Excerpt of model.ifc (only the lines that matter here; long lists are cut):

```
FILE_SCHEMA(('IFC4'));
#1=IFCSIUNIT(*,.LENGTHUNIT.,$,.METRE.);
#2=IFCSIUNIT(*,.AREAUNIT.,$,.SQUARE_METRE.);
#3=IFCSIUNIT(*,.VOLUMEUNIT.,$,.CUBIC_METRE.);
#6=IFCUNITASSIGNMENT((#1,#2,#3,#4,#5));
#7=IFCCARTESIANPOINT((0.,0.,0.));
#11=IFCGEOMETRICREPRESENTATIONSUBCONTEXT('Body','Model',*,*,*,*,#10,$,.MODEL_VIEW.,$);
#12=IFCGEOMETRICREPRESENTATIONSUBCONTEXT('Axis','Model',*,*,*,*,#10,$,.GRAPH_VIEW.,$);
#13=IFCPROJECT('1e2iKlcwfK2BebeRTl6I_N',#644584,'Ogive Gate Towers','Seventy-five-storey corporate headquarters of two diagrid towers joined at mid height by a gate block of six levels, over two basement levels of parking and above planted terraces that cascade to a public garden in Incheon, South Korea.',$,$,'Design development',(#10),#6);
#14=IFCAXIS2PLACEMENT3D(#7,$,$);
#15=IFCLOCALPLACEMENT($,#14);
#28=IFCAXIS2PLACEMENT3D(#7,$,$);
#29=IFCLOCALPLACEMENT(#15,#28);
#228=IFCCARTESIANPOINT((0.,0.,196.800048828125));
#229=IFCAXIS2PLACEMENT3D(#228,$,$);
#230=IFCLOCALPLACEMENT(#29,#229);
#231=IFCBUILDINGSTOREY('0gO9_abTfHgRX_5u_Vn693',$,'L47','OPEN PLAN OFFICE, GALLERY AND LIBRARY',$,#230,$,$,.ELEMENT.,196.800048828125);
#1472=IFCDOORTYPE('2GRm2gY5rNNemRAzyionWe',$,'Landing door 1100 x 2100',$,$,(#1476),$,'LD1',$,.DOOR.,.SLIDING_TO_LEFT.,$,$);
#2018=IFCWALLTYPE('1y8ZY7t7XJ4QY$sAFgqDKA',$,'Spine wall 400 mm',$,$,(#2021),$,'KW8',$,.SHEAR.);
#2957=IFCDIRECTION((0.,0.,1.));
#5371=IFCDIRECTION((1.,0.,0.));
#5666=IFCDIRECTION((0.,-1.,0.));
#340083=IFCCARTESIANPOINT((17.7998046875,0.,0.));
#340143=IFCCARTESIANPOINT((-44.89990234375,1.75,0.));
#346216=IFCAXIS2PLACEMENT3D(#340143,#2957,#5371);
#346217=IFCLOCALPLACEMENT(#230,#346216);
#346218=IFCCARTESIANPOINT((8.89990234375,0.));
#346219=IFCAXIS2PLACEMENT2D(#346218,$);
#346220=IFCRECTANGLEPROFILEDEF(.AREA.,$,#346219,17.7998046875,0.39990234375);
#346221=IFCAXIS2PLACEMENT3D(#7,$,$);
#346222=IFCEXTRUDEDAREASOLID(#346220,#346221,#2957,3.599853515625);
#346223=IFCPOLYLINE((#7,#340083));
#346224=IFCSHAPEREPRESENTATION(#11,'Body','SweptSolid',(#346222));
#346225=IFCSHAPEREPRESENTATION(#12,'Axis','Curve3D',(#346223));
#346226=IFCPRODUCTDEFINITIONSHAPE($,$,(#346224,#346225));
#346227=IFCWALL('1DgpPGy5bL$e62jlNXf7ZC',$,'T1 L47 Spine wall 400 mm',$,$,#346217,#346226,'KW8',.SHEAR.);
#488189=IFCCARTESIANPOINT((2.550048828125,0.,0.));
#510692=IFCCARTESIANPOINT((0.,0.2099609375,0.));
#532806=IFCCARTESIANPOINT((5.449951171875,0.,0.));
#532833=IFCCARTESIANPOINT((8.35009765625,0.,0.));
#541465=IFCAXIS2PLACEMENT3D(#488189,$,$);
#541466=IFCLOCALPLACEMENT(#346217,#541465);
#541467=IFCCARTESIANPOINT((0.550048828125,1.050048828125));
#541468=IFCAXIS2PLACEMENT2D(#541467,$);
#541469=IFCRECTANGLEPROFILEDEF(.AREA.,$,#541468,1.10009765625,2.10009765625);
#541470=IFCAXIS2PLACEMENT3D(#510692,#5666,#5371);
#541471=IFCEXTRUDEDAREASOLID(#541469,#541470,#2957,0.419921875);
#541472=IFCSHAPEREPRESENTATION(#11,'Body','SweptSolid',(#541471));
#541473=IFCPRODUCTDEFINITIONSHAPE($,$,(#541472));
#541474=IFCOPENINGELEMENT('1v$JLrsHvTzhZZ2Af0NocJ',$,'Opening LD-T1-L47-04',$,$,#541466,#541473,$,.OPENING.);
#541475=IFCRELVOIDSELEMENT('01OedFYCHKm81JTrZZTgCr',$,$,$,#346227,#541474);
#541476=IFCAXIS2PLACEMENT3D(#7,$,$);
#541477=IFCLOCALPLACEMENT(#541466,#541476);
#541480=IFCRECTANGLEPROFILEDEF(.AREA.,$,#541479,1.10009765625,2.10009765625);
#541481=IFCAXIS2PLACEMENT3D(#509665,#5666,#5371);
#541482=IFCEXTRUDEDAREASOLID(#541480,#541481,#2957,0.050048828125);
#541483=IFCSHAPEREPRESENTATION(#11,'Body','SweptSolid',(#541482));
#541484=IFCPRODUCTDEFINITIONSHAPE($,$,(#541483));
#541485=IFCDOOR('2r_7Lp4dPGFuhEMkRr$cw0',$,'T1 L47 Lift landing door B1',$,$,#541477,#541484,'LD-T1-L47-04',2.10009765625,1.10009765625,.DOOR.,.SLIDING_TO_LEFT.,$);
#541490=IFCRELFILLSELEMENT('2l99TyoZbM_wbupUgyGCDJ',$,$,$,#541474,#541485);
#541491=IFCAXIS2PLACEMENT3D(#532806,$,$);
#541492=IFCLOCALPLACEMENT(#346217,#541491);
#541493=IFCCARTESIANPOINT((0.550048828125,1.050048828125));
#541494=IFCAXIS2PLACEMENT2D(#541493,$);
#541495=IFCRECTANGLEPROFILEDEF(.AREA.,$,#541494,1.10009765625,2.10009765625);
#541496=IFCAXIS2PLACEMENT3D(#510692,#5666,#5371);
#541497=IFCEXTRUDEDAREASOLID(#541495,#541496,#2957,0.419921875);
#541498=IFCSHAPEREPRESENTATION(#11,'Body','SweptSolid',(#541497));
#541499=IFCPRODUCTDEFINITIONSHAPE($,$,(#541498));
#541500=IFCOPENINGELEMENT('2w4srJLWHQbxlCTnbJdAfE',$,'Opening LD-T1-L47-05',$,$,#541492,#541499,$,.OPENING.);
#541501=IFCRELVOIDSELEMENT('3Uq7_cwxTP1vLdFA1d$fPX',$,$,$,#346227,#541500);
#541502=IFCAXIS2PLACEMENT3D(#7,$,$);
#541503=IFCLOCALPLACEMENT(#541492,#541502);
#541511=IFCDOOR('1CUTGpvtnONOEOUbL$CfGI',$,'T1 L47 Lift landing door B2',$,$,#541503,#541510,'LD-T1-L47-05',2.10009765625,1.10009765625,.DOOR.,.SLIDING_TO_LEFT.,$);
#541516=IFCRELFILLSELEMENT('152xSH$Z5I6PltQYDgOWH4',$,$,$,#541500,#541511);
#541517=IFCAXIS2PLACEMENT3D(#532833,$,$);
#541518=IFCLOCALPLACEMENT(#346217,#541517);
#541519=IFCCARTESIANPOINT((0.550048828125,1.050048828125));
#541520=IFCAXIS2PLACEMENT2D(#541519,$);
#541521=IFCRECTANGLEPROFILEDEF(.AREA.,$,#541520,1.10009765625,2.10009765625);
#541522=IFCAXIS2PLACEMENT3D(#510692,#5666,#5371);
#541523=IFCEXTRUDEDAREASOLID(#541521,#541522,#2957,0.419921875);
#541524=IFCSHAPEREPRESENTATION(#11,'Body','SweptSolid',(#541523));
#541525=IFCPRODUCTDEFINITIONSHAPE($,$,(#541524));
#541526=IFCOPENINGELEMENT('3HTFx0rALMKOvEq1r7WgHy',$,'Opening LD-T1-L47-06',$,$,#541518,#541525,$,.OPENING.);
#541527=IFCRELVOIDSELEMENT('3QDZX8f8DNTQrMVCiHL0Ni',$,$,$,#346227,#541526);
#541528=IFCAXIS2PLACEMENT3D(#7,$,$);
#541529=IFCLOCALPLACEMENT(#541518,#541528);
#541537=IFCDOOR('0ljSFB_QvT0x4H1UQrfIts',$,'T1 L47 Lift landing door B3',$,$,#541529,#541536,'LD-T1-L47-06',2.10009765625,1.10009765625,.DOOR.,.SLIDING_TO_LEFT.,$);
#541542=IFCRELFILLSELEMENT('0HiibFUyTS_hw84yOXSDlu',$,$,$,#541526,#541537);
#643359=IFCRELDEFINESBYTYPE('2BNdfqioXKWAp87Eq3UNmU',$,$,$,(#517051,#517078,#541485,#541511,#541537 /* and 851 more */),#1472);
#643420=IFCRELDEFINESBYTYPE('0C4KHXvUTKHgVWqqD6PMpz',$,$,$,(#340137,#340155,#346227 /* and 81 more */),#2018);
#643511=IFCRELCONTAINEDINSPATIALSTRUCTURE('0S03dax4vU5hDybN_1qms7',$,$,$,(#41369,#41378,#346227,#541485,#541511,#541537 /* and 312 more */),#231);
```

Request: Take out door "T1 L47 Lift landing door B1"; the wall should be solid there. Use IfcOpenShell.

```python
import ifcopenshell
import ifcopenshell.api.feature
import ifcopenshell.api.root
import ifcopenshell.geom
import ifcopenshell.util.shape

model = ifcopenshell.open("model.ifc")
settings = ifcopenshell.geom.settings()


def volume(element):
    """Net volume in cubic metres, openings subtracted."""
    shape = ifcopenshell.geom.create_shape(settings, element)
    return ifcopenshell.util.shape.get_volume(shape.geometry)


door = model.by_guid("2r_7Lp4dPGFuhEMkRr$cw0")
opening = door.FillsVoids[0].RelatingOpeningElement
wall = opening.VoidsElements[0].RelatingBuildingElement
before = volume(wall)

ifcopenshell.api.root.remove_product(model, product=door)
ifcopenshell.api.feature.remove_feature(model, feature=opening)

after = volume(wall)

print(f"wall volume {before:.3f} -> {after:.3f} m3")

model.write("model-out.ifc")
```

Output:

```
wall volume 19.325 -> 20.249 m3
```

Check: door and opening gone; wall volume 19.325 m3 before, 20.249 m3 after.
